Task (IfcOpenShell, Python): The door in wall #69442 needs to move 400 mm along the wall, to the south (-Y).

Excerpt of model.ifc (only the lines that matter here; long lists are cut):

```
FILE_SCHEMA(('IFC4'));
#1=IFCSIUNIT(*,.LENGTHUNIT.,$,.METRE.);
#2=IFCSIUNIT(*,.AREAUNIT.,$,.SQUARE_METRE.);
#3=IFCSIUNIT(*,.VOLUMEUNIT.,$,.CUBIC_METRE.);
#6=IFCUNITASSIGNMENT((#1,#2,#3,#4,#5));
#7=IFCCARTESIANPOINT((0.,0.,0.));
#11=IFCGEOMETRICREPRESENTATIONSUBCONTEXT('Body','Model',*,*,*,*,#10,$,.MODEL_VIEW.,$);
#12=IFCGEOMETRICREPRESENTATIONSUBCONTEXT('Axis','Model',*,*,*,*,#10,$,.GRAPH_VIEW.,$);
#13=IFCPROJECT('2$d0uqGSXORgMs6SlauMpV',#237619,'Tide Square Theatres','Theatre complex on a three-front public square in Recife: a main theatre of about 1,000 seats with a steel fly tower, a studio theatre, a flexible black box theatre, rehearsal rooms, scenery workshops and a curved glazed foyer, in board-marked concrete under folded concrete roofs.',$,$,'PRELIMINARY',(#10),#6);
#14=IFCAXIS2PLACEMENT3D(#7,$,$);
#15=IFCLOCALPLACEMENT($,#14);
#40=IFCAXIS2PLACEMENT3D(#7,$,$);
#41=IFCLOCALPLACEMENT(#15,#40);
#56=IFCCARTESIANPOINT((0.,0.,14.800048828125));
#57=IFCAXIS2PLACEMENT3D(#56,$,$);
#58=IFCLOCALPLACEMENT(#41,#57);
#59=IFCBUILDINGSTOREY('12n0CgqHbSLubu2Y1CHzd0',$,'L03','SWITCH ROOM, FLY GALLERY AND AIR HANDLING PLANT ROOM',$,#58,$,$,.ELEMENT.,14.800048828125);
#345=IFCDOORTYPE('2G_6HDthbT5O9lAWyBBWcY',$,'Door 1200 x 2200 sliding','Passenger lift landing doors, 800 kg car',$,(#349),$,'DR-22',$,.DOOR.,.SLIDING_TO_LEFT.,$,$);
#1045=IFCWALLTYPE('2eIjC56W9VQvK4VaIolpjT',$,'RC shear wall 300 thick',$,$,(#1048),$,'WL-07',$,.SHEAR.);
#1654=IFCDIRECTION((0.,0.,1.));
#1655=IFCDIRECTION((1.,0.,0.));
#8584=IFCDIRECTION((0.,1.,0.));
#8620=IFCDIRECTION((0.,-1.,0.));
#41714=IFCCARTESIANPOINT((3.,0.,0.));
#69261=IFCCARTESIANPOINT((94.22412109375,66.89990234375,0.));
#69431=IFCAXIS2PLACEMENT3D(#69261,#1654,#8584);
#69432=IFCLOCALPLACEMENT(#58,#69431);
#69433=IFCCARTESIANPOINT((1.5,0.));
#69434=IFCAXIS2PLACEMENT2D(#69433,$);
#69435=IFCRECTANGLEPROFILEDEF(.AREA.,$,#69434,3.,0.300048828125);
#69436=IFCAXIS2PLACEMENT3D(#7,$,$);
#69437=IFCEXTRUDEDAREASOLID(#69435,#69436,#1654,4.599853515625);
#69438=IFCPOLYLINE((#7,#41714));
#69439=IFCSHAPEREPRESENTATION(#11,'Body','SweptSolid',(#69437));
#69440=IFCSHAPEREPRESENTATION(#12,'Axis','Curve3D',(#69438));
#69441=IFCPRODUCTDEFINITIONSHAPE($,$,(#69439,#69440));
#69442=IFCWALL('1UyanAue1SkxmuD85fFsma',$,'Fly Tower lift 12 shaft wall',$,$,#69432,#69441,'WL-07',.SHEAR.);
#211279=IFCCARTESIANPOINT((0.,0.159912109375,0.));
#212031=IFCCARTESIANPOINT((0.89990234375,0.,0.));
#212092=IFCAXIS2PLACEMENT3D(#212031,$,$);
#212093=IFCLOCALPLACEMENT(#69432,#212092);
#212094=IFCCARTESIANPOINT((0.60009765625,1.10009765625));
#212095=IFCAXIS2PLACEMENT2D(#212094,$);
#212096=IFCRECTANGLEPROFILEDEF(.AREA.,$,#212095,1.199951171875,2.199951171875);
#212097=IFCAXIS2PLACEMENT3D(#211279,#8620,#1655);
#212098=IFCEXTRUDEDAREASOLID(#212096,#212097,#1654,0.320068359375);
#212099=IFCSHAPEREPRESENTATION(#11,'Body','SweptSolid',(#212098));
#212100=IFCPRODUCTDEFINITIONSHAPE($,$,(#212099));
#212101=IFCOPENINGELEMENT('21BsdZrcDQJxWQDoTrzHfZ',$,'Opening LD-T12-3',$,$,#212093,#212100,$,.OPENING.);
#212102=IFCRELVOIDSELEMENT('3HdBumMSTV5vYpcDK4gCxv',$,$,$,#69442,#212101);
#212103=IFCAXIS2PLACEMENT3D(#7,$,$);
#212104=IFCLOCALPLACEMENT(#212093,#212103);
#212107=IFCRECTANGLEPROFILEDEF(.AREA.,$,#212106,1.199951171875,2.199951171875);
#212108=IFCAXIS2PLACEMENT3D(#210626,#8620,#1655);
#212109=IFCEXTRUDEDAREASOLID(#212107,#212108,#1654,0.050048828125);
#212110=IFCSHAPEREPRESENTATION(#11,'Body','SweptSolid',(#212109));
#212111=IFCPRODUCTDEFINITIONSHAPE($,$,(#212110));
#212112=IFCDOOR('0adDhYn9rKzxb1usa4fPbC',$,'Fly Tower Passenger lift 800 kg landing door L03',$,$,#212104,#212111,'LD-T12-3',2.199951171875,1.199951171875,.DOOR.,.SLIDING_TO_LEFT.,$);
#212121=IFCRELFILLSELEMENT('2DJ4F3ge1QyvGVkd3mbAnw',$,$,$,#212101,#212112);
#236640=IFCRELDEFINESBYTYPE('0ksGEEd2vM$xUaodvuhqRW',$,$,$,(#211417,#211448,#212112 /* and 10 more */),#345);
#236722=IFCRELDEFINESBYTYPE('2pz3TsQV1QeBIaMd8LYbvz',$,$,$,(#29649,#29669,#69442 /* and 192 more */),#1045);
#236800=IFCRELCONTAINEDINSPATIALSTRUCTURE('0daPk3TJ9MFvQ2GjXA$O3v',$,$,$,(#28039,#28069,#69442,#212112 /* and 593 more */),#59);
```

```python
import ifcopenshell
import ifcopenshell.api.geometry
import ifcopenshell.util.placement
import ifcopenshell.util.unit

model = ifcopenshell.open("model.ifc")
unit_scale = ifcopenshell.util.unit.calculate_unit_scale(model)

door = model.by_id(212112)
opening = door.FillsVoids[0].RelatingOpeningElement
wall = opening.VoidsElements[0].RelatingBuildingElement

wall_matrix = ifcopenshell.util.placement.get_local_placement(wall.ObjectPlacement)
shift = wall_matrix[:3, 0] * -0.4 / unit_scale
before = ifcopenshell.util.placement.get_local_placement(door.ObjectPlacement)[:3, 3].copy()

# The door is placed relative to its opening, so it follows when the opening moves.
matrix = ifcopenshell.util.placement.get_local_placement(opening.ObjectPlacement)
matrix[:3, 3] += shift
ifcopenshell.api.geometry.edit_object_placement(
    model, product=opening, matrix=matrix, is_si=False, should_transform_children=True
)

after = ifcopenshell.util.placement.get_local_placement(door.ObjectPlacement)[:3, 3]
print("door moved by", (after - before).round(3) + 0.0)

model.write("model_edited.ifc")
```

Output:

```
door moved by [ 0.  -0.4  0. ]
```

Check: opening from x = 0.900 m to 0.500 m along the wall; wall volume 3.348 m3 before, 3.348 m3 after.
